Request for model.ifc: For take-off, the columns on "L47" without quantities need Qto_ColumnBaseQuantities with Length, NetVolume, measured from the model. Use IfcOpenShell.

First a look at what the model holds.

```python
import ifcopenshell
import ifcopenshell.util.element
import ifcopenshell.util.unit

model = ifcopenshell.open("model.ifc")
print(model.schema)
for unit_type in ("LENGTHUNIT", "AREAUNIT", "VOLUMEUNIT"):
    print(unit_type, ifcopenshell.util.unit.calculate_unit_scale(model, unit_type))
storey = next(s for s in model.by_type("IfcBuildingStorey") if s.Name == "L47")
columns = [e for e in ifcopenshell.util.element.get_decomposition(storey) if e.is_a("IfcColumn")]
for e in sorted(columns, key=lambda e: e.id()):
    print(e.id(), e.is_a(), e.Name, list(ifcopenshell.util.element.get_psets(e, qtos_only=True)), sep=" | ")
```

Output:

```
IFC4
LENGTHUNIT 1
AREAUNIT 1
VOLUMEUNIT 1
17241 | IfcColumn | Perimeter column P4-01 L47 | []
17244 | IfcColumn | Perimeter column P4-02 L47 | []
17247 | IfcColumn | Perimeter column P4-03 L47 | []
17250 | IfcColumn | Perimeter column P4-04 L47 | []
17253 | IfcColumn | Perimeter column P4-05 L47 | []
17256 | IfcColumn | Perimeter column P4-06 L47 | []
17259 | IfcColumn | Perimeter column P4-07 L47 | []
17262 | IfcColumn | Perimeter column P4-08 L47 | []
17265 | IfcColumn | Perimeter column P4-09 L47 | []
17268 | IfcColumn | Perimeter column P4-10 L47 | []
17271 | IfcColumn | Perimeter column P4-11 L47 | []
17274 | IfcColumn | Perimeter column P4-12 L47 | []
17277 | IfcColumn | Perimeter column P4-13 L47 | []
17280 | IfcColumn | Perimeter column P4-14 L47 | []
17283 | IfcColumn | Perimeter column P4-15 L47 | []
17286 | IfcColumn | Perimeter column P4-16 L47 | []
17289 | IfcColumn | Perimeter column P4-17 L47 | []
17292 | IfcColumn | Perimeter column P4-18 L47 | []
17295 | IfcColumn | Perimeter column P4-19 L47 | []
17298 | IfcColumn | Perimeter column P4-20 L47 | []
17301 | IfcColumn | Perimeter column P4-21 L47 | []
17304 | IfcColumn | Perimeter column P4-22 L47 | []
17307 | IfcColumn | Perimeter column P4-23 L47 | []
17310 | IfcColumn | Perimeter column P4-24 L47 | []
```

```python
import ifcopenshell
import ifcopenshell.api.pset
import ifcopenshell.geom
import ifcopenshell.util.element
import ifcopenshell.util.shape
import ifcopenshell.util.unit

model = ifcopenshell.open("model.ifc")
unit_scale = ifcopenshell.util.unit.calculate_unit_scale(model)
volume_scale = ifcopenshell.util.unit.calculate_unit_scale(model, "VOLUMEUNIT")
settings = ifcopenshell.geom.settings()

storey = next(s for s in model.by_type("IfcBuildingStorey") if s.Name == "L47")
columns = [e for e in ifcopenshell.util.element.get_decomposition(storey) if e.is_a("IfcColumn")]

for e in sorted(columns, key=lambda e: e.id()):
    if ifcopenshell.util.element.get_psets(e, qtos_only=True, should_inherit=False):
        continue
    # Geometry comes back in metres, in the element's own axes.
    shape = ifcopenshell.geom.create_shape(settings, e)
    values = {
        "Length": ifcopenshell.util.shape.get_z(shape.geometry) / unit_scale,
        "NetVolume": ifcopenshell.util.shape.get_volume(shape.geometry) / volume_scale,
    }
    qto = ifcopenshell.api.pset.add_qto(model, product=e, name="Qto_ColumnBaseQuantities")
    ifcopenshell.api.pset.edit_qto(model, qto=qto, properties=values)
    print(e.id(), {k: round(v, 3) for k, v in values.items()})

model.write("model_edited.ifc")
```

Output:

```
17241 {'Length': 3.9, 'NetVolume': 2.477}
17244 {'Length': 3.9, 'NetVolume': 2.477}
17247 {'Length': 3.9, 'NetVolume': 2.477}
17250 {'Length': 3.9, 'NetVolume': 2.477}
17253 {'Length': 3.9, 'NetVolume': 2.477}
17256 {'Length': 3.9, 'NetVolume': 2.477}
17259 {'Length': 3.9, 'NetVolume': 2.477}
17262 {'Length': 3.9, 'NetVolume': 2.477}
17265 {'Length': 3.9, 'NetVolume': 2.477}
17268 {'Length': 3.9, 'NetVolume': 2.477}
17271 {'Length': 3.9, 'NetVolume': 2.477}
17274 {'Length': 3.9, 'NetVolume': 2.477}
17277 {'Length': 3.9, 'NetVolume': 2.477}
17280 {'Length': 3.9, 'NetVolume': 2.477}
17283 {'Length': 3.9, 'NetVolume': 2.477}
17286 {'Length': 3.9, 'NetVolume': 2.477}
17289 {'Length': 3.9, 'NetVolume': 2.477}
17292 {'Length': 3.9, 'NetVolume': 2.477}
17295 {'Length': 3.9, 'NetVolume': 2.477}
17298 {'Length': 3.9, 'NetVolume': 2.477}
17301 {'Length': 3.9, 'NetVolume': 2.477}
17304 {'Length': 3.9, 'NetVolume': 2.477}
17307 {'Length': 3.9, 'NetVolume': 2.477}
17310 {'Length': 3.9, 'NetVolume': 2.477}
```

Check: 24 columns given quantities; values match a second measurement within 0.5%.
